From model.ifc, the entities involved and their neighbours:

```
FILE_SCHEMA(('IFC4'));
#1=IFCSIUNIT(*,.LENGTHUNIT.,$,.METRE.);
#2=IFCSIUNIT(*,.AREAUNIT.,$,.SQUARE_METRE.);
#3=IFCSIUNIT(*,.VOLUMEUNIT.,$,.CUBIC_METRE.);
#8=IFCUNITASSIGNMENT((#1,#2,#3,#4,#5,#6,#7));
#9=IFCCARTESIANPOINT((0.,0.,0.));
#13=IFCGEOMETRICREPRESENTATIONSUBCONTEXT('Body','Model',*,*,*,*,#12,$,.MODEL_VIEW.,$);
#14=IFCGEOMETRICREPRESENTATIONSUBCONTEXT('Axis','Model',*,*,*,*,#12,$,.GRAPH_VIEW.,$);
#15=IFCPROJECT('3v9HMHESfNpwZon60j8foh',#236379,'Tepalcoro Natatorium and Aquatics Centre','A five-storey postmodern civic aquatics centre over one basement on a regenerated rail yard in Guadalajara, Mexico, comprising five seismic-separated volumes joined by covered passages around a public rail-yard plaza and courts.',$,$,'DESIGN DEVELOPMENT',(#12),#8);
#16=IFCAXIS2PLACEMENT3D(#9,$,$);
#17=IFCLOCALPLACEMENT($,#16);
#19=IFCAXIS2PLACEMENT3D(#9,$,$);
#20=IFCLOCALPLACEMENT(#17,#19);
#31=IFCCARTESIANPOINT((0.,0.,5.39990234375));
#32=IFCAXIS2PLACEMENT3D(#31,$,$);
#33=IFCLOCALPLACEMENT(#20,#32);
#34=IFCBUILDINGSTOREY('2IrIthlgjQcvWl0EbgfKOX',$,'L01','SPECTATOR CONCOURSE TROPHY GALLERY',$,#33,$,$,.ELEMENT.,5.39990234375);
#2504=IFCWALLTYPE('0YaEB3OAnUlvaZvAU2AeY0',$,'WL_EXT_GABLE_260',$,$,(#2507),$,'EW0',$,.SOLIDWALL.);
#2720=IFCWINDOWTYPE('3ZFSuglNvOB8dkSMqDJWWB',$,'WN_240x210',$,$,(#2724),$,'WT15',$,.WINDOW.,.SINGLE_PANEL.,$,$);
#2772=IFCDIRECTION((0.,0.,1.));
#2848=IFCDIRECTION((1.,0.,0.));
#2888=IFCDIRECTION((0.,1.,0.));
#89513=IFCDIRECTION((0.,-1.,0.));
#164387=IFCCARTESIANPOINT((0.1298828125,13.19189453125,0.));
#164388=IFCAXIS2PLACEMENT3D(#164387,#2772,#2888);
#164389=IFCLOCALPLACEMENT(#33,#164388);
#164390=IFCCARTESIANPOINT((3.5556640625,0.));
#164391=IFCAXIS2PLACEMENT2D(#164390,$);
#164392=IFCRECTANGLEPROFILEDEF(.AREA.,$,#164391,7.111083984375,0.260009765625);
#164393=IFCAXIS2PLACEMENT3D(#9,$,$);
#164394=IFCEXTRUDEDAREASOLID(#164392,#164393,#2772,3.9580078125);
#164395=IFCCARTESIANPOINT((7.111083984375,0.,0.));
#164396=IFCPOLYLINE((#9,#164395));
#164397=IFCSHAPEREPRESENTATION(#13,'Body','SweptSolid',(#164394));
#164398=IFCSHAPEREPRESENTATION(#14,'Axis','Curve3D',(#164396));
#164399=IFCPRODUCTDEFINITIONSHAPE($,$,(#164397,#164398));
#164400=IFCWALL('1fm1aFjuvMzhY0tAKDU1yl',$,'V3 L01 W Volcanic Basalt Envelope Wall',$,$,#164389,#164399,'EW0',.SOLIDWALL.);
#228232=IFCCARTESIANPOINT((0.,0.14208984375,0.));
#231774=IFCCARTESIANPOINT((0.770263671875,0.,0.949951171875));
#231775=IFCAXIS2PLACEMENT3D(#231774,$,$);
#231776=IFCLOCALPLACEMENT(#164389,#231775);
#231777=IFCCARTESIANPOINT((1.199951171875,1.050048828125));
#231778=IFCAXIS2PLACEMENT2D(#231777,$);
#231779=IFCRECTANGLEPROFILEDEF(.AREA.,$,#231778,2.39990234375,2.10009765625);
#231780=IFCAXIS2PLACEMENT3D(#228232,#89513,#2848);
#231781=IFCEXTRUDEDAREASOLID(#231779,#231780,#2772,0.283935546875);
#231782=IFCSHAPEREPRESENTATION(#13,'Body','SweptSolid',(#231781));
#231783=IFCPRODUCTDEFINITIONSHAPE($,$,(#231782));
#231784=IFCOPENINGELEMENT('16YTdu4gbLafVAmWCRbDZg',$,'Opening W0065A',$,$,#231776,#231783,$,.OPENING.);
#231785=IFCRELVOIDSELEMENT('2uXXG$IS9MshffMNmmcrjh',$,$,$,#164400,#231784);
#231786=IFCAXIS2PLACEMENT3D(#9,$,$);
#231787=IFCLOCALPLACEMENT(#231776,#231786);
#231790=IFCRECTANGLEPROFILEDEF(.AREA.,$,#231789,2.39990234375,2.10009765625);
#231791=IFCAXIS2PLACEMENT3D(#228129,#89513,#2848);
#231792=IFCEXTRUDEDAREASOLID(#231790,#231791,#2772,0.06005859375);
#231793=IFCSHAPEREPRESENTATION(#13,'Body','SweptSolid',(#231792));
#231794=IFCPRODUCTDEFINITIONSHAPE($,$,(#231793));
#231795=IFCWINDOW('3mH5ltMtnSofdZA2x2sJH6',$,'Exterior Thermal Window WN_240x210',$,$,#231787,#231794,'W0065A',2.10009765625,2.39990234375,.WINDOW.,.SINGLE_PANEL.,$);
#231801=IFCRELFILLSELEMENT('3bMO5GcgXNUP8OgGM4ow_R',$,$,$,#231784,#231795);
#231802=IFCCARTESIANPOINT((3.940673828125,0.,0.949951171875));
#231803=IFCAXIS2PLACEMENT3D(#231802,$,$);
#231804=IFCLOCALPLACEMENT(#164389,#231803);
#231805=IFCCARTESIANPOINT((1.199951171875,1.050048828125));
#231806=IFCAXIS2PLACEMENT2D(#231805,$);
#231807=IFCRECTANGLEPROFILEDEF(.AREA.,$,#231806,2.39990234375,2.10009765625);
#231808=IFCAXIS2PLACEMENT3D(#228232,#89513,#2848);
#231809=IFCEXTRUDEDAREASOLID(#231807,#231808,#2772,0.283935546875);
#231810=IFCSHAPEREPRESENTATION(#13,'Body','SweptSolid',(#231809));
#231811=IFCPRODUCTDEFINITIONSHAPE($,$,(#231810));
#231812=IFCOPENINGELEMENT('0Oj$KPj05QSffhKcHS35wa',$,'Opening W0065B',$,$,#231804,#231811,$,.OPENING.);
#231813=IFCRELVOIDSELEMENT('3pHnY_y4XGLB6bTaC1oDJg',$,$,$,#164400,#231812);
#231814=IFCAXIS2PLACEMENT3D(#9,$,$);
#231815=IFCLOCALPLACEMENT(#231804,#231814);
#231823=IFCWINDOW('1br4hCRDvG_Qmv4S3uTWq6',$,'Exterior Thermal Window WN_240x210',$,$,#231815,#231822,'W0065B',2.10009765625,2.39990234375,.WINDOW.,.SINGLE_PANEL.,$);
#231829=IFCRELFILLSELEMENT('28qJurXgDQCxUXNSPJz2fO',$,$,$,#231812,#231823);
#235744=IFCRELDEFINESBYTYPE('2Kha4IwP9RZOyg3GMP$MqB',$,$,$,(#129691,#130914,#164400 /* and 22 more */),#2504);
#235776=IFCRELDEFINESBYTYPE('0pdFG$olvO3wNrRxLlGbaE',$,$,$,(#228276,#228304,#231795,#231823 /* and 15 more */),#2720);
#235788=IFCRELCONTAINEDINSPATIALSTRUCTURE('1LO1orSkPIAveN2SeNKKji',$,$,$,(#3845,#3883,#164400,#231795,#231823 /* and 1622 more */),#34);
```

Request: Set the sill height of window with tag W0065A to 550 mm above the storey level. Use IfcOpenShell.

```python
import numpy as np
import ifcopenshell
import ifcopenshell.api.geometry
import ifcopenshell.geom
import ifcopenshell.util.element
import ifcopenshell.util.placement
import ifcopenshell.util.shape
import ifcopenshell.util.unit

model = ifcopenshell.open("model.ifc")
unit_scale = ifcopenshell.util.unit.calculate_unit_scale(model)

window = model.by_guid("3mH5ltMtnSofdZA2x2sJH6")
opening = window.FillsVoids[0].RelatingOpeningElement
storey = ifcopenshell.util.element.get_container(window, ifc_class="IfcBuildingStorey")
level = ifcopenshell.util.placement.get_local_placement(storey.ObjectPlacement)[2, 3]

# The opening's origin need not be at the sill, so measure its lowest point.
shape = ifcopenshell.geom.create_shape(ifcopenshell.geom.settings(), opening)
bottom = ifcopenshell.util.shape.get_shape_bottom_elevation(shape, shape.geometry) / unit_scale
dz = level + 0.55 - bottom

shift = np.array([0.0, 0.0, dz])
# The window is placed relative to its opening, so it follows when the opening moves.
matrix = ifcopenshell.util.placement.get_local_placement(opening.ObjectPlacement)
matrix[:3, 3] += shift
ifcopenshell.api.geometry.edit_object_placement(
    model, product=opening, matrix=matrix, is_si=False, should_transform_children=True
)

print(f"moved by {dz * unit_scale:+.3f} m")

model.write("model_updated.ifc")
```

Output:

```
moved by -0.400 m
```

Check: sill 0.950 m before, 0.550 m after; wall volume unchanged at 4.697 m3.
